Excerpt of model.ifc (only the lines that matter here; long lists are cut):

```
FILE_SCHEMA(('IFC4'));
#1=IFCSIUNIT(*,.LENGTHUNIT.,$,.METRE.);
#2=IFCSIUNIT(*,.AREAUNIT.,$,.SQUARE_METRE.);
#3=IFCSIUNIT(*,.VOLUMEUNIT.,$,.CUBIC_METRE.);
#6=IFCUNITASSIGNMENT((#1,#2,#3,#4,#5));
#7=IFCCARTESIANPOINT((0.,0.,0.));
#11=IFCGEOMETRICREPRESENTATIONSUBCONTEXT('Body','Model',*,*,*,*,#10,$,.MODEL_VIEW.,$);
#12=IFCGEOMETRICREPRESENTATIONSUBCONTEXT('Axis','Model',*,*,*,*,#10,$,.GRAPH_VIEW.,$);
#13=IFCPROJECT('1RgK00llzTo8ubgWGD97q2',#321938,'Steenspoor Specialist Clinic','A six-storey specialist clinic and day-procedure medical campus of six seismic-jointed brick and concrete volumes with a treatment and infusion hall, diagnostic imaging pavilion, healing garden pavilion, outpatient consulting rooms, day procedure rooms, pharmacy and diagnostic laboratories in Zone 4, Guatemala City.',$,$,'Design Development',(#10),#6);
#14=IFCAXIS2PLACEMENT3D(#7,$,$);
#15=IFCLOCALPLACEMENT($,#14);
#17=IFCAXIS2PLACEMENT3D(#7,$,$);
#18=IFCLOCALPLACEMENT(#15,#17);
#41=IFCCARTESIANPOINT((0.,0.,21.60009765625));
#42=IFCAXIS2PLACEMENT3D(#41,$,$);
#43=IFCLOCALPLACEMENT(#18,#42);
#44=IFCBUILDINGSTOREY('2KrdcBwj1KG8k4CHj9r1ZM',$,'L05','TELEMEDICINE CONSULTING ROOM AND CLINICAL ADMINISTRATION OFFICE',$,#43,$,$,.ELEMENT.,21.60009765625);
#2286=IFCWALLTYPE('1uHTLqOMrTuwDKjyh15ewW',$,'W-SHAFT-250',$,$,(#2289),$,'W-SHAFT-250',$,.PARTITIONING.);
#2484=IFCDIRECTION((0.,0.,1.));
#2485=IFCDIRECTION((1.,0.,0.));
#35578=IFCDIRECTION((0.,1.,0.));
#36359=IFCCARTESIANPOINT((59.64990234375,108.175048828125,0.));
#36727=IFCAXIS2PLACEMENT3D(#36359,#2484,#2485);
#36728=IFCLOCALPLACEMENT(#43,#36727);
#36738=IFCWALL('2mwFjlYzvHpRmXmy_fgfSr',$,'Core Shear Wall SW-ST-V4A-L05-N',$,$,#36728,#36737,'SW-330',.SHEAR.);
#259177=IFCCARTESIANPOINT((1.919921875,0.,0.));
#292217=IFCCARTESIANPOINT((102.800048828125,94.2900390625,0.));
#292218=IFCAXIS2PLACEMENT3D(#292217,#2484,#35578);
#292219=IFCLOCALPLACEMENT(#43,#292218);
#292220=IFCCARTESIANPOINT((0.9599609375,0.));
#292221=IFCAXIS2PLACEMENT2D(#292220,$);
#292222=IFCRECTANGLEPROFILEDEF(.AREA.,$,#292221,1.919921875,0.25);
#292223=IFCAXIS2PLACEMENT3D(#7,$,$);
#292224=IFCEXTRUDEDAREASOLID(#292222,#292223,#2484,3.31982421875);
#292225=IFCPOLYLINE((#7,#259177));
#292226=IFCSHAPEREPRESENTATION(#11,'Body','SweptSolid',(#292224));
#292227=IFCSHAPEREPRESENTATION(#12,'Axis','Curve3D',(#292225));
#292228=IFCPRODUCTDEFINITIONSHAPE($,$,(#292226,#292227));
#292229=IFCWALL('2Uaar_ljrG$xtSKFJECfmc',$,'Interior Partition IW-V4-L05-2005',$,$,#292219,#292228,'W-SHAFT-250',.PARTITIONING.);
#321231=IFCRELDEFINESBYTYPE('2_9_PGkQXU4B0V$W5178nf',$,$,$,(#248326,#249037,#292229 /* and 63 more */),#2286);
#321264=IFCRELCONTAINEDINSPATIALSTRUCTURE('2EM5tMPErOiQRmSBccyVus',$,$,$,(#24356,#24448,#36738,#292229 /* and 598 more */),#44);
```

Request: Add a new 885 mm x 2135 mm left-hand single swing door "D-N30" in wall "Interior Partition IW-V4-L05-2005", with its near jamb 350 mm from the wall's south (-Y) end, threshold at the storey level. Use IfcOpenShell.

```python
import numpy as np
import ifcopenshell
import ifcopenshell.api.feature
import ifcopenshell.api.geometry
import ifcopenshell.api.root
import ifcopenshell.api.spatial
import ifcopenshell.geom
import ifcopenshell.util.element
import ifcopenshell.util.placement
import ifcopenshell.util.representation
import ifcopenshell.util.shape
import ifcopenshell.util.unit

model = ifcopenshell.open("model.ifc")
unit_scale = ifcopenshell.util.unit.calculate_unit_scale(model)
settings = ifcopenshell.geom.settings()


def volume(element):
    """Net volume in cubic metres, openings subtracted."""
    shape = ifcopenshell.geom.create_shape(settings, element)
    return ifcopenshell.util.shape.get_volume(shape.geometry)


wall = model.by_guid("2Uaar_ljrG$xtSKFJECfmc")
storey = ifcopenshell.util.element.get_container(wall, ifc_class="IfcBuildingStorey")
context = ifcopenshell.util.representation.get_context(model, "Model", "Body", "MODEL_VIEW")
before = volume(wall)

width, height, from_end, sill = 0.885, 2.135, 0.35, 0.0  # metres

# The wall runs along its own X axis, and the end named is its -X end.
wall_shape = ifcopenshell.geom.create_shape(settings, wall)
x, y, z = ifcopenshell.util.shape.get_vertices(wall_shape.geometry).T
start = x.min() + from_end
face, thickness = float(y.min()), float(y.max() - y.min())
wall_matrix = ifcopenshell.util.placement.get_local_placement(wall.ObjectPlacement)
level = ifcopenshell.util.placement.get_local_placement(storey.ObjectPlacement)[2, 3]


def in_wall(x, y):
    """Placement at x, y metres in the wall's axes, at sill height."""
    matrix = wall_matrix.copy()
    matrix[:, 3] = wall_matrix @ np.array([x / unit_scale, y / unit_scale, 0.0, 1.0])
    matrix[2, 3] = level + sill / unit_scale
    return matrix


# Opening: a box that overshoots both wall faces by 50 mm.
opening = ifcopenshell.api.root.create_entity(model, ifc_class="IfcOpeningElement", predefined_type="OPENING")
box = ifcopenshell.api.geometry.add_wall_representation(
    model, context=context, length=width, height=height, thickness=thickness + 0.1
)
ifcopenshell.api.geometry.assign_representation(model, product=opening, representation=box)
ifcopenshell.api.geometry.edit_object_placement(model, product=opening, matrix=in_wall(start, face - 0.05), is_si=False)
ifcopenshell.api.feature.add_feature(model, feature=opening, element=wall)

door = ifcopenshell.api.root.create_entity(model, ifc_class="IfcDoor", name="D-N30", predefined_type="DOOR")
door.OverallWidth, door.OverallHeight = width / unit_scale, height / unit_scale
door.OperationType = "SINGLE_SWING_LEFT"
body = ifcopenshell.api.geometry.add_door_representation(
    model,
    context=context,
    overall_width=door.OverallWidth,
    overall_height=door.OverallHeight,
    operation_type="SINGLE_SWING_LEFT",
    lining_properties={"LiningDepth": thickness / unit_scale, "ThresholdDepth": thickness / unit_scale},
)
ifcopenshell.api.geometry.assign_representation(model, product=door, representation=body)
ifcopenshell.api.spatial.assign_container(model, products=[door], relating_structure=storey)
ifcopenshell.api.feature.add_filling(model, opening=opening, element=door)

# The lining spans the wall, so the door starts at the wall face.
ifcopenshell.api.geometry.edit_object_placement(model, product=door, matrix=in_wall(start, face), is_si=False)

after = volume(wall)

print(f"wall volume {before:.3f} -> {after:.3f} m3")

model.write("model_updated.ifc")
```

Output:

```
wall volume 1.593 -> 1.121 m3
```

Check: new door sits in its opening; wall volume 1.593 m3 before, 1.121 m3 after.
